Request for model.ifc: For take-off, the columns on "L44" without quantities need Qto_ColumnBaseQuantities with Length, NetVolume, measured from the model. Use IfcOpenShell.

First a look at what the model holds.

```python
import ifcopenshell
import ifcopenshell.util.element
import ifcopenshell.util.unit

model = ifcopenshell.open("model.ifc")
print(model.schema)
for unit_type in ("LENGTHUNIT", "AREAUNIT", "VOLUMEUNIT"):
    print(unit_type, ifcopenshell.util.unit.calculate_unit_scale(model, unit_type))
storey = next(s for s in model.by_type("IfcBuildingStorey") if s.Name == "L44")
columns = [e for e in ifcopenshell.util.element.get_decomposition(storey) if e.is_a("IfcColumn")]
for e in sorted(columns, key=lambda e: e.id()):
    print(e.id(), e.is_a(), e.Name, list(ifcopenshell.util.element.get_psets(e, qtos_only=True)), sep=" | ")
```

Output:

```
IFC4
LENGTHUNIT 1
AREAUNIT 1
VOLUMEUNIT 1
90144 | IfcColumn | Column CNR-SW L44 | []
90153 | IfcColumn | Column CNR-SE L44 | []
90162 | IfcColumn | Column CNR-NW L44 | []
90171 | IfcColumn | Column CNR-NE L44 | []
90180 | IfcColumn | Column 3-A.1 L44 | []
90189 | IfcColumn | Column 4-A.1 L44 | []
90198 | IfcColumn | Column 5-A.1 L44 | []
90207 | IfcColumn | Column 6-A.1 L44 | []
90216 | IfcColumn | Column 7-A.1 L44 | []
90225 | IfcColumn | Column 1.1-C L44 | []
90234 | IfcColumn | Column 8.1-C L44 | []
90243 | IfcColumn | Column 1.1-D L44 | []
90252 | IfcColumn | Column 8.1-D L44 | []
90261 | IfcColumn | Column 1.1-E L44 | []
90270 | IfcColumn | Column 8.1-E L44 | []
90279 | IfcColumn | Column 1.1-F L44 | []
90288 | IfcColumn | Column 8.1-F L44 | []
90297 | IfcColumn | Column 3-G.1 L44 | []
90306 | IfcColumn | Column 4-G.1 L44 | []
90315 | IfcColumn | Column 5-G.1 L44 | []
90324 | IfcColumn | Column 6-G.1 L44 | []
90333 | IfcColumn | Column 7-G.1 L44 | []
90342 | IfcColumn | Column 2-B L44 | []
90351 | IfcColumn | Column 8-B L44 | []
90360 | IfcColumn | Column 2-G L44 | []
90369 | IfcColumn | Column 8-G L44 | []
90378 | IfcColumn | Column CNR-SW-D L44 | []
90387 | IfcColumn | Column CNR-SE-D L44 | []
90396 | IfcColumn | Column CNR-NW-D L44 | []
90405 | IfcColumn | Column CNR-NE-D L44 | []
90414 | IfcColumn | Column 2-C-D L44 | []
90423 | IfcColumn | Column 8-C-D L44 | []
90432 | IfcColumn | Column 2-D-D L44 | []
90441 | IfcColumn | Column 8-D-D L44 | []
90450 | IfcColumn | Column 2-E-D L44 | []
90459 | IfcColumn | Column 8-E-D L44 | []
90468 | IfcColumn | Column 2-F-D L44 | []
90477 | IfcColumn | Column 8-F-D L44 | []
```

```python
import ifcopenshell
import ifcopenshell.api.pset
import ifcopenshell.geom
import ifcopenshell.util.element
import ifcopenshell.util.shape
import ifcopenshell.util.unit

model = ifcopenshell.open("model.ifc")
unit_scale = ifcopenshell.util.unit.calculate_unit_scale(model)
volume_scale = ifcopenshell.util.unit.calculate_unit_scale(model, "VOLUMEUNIT")
settings = ifcopenshell.geom.settings()

storey = next(s for s in model.by_type("IfcBuildingStorey") if s.Name == "L44")
columns = [e for e in ifcopenshell.util.element.get_decomposition(storey) if e.is_a("IfcColumn")]

for e in sorted(columns, key=lambda e: e.id()):
    if ifcopenshell.util.element.get_psets(e, qtos_only=True, should_inherit=False):
        continue
    # Geometry comes back in metres, in the element's own axes.
    shape = ifcopenshell.geom.create_shape(settings, e)
    values = {
        "Length": ifcopenshell.util.shape.get_z(shape.geometry) / unit_scale,
        "NetVolume": ifcopenshell.util.shape.get_volume(shape.geometry) / volume_scale,
    }
    qto = ifcopenshell.api.pset.add_qto(model, product=e, name="Qto_ColumnBaseQuantities")
    ifcopenshell.api.pset.edit_qto(model, qto=qto, properties=values)
    print(e.id(), {k: round(v, 3) for k, v in values.items()})

model.write("model-out.ifc")
```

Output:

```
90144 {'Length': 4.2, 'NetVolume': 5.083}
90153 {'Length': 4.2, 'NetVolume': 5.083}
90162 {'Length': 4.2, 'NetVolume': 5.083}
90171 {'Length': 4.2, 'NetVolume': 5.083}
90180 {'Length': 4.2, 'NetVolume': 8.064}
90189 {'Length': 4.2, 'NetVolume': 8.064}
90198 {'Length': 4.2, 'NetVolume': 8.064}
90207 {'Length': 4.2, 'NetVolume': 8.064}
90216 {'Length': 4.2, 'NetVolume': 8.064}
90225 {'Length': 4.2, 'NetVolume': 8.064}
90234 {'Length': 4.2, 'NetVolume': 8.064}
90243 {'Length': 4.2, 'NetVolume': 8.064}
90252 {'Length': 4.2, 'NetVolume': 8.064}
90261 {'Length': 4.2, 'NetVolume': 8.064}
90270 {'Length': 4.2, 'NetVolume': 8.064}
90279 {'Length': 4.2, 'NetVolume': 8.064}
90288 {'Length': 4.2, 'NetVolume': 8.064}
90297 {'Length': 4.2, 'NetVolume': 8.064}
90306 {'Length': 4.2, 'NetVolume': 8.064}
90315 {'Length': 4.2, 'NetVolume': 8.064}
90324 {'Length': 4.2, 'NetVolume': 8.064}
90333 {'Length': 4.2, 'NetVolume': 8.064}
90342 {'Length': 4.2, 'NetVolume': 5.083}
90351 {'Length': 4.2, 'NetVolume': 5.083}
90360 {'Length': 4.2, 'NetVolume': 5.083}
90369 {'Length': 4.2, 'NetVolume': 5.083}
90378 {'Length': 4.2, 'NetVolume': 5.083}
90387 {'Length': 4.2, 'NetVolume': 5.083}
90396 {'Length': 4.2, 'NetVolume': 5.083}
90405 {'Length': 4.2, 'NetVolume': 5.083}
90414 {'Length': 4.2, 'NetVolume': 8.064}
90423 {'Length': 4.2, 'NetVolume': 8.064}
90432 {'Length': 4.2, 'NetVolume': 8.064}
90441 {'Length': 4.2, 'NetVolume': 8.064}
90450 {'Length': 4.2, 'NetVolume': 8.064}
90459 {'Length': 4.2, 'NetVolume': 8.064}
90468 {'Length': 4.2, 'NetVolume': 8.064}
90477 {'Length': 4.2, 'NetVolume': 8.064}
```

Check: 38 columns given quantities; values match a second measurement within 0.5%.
